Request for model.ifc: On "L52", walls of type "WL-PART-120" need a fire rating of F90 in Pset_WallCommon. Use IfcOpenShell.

First a look at what the model holds.

```python
import ifcopenshell
import ifcopenshell.util.element

model = ifcopenshell.open("model.ifc")
print(model.schema)
storey = next(s for s in model.by_type("IfcBuildingStorey") if s.Name == "L52")
walls = [e for e in ifcopenshell.util.element.get_decomposition(storey) if e.is_a("IfcWall")]
seen = {}
for e in walls:
    element_type = ifcopenshell.util.element.get_type(e)
    key = (element_type.Name if element_type != e and element_type else None, ifcopenshell.util.element.get_pset(e, "Pset_WallCommon", "FireRating"))
    seen[key] = seen.get(key, 0) + 1
for (name, value), count in sorted(seen.items(), key=str):
    print(count, "x", name, "|", value)
```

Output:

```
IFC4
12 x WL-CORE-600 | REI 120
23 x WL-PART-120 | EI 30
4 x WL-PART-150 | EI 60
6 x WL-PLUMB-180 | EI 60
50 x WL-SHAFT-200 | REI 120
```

```python
import ifcopenshell
import ifcopenshell.api.pset
import ifcopenshell.util.element

model = ifcopenshell.open("model.ifc")

storey = next(s for s in model.by_type("IfcBuildingStorey") if s.Name == "L52")
walls = [e for e in ifcopenshell.util.element.get_decomposition(storey) if e.is_a("IfcWall")]

count = 0
for e in walls:
    element_type = ifcopenshell.util.element.get_type(e)
    if element_type in (None, e) or element_type.Name != "WL-PART-120":
        continue
    # add_pset returns the element's existing set when there is one.
    pset = ifcopenshell.api.pset.add_pset(model, product=e, name="Pset_WallCommon")
    ifcopenshell.api.pset.edit_pset(model, pset=pset, properties={"FireRating": "F90"})
    count += 1

print(count, "walls updated")

model.write("model-out.ifc")
```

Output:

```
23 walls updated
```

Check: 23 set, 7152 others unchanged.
